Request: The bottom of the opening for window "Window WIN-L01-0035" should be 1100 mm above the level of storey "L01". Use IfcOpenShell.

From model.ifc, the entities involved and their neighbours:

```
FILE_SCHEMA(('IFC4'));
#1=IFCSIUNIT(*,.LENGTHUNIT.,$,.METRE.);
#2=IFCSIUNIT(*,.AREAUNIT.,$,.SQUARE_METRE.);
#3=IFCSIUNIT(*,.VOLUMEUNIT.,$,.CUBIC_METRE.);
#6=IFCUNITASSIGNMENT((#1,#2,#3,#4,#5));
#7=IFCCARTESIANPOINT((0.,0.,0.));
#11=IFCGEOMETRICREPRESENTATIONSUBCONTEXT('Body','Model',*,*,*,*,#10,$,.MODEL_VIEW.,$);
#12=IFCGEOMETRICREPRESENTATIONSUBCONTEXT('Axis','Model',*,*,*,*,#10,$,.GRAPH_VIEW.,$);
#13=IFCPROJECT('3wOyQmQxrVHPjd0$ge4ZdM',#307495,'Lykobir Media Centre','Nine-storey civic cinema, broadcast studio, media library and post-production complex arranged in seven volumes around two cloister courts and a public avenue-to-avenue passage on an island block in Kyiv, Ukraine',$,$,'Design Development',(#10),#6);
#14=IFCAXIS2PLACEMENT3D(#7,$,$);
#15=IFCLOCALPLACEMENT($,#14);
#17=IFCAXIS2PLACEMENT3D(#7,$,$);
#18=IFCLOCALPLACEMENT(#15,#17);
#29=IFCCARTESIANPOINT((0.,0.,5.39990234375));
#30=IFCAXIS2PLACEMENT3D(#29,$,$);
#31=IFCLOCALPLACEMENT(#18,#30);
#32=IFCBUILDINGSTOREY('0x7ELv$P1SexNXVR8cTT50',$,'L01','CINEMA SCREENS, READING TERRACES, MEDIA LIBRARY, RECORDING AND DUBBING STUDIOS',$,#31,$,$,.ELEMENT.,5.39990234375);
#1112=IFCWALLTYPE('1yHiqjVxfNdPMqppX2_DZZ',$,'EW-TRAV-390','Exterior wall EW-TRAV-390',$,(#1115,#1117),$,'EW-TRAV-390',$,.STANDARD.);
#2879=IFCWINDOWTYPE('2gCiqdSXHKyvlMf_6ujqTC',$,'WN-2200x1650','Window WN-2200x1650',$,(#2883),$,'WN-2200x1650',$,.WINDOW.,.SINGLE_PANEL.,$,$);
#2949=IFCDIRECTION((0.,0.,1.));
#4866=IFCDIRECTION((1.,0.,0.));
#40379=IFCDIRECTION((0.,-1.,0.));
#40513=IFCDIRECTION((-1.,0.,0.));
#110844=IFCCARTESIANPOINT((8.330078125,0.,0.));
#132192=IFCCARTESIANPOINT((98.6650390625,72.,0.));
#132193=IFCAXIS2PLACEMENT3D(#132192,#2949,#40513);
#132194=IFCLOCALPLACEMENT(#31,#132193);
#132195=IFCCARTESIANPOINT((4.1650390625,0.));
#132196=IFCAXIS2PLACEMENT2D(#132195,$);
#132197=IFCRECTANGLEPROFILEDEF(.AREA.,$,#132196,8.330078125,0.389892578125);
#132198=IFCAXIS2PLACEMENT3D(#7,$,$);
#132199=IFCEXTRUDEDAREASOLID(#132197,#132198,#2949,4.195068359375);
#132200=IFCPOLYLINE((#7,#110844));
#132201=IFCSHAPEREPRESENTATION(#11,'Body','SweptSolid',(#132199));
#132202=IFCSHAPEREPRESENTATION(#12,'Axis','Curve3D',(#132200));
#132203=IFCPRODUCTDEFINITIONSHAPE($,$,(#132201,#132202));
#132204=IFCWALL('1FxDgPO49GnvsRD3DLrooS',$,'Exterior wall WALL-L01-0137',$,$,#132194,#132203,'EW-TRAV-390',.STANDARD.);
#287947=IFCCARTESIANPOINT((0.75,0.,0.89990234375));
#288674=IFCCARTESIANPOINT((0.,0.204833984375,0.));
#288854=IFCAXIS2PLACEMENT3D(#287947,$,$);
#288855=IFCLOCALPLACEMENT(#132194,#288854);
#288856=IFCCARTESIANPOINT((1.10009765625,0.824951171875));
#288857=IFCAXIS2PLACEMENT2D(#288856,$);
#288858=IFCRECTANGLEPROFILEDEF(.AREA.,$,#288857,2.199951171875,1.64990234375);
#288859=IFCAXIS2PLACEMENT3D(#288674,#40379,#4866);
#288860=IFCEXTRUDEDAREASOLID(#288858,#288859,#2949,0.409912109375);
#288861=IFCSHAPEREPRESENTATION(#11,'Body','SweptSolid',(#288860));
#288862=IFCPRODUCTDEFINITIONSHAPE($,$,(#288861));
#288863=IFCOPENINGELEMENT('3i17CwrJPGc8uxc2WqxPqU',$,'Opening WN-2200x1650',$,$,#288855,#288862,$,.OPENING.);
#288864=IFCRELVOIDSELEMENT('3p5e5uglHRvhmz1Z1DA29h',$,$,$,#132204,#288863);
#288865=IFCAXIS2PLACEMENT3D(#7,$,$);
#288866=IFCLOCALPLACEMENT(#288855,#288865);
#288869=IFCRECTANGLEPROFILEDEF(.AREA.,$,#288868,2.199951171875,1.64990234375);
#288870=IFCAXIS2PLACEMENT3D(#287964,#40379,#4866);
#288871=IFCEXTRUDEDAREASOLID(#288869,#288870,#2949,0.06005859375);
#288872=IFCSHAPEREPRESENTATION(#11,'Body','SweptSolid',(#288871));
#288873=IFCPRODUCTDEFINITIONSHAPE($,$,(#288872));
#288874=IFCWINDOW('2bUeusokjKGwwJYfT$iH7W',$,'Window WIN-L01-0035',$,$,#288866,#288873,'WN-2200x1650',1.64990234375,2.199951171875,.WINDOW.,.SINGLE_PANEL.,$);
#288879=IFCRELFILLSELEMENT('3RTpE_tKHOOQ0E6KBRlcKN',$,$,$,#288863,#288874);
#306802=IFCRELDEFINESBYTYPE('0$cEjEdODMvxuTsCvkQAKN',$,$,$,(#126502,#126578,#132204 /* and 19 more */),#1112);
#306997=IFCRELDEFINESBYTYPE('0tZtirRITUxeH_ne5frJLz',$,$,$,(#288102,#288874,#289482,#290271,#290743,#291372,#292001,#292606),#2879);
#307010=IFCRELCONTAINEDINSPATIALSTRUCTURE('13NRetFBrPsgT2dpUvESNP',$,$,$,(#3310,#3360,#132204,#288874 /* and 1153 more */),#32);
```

```python
import numpy as np
import ifcopenshell
import ifcopenshell.api.geometry
import ifcopenshell.geom
import ifcopenshell.util.element
import ifcopenshell.util.placement
import ifcopenshell.util.shape
import ifcopenshell.util.unit

model = ifcopenshell.open("model.ifc")
unit_scale = ifcopenshell.util.unit.calculate_unit_scale(model)

window = model.by_guid("2bUeusokjKGwwJYfT$iH7W")
opening = window.FillsVoids[0].RelatingOpeningElement
storey = ifcopenshell.util.element.get_container(window, ifc_class="IfcBuildingStorey")
level = ifcopenshell.util.placement.get_local_placement(storey.ObjectPlacement)[2, 3]

# The opening's origin need not be at the sill, so measure its lowest point.
shape = ifcopenshell.geom.create_shape(ifcopenshell.geom.settings(), opening)
bottom = ifcopenshell.util.shape.get_shape_bottom_elevation(shape, shape.geometry) / unit_scale
dz = level + 1.1 / unit_scale - bottom

shift = np.array([0.0, 0.0, dz])
# The window is placed relative to its opening, so it follows when the opening moves.
matrix = ifcopenshell.util.placement.get_local_placement(opening.ObjectPlacement)
matrix[:3, 3] += shift
ifcopenshell.api.geometry.edit_object_placement(
    model, product=opening, matrix=matrix, is_si=False, should_transform_children=True
)

print(f"moved by {dz * unit_scale:+.3f} m")

model.write("model_rev.ifc")
```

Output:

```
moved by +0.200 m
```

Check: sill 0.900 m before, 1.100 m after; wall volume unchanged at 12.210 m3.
